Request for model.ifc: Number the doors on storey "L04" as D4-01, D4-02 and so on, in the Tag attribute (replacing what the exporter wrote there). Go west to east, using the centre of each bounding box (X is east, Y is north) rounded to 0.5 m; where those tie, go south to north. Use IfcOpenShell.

First a look at what the model holds.

```python
import ifcopenshell
import ifcopenshell.util.element
import ifcopenshell.util.placement

model = ifcopenshell.open("model.ifc")
print(model.schema)
storey = next(s for s in model.by_type("IfcBuildingStorey") if s.Name == "L04")
doors = [e for e in ifcopenshell.util.element.get_decomposition(storey) if e.is_a("IfcDoor")]
for e in sorted(doors, key=lambda e: e.id()):
    origin = ifcopenshell.util.placement.get_local_placement(e.ObjectPlacement)[:3, 3]
    print(e.id(), e.Tag, e.Name, origin.round(2) + 0.0, sep=" | ")
```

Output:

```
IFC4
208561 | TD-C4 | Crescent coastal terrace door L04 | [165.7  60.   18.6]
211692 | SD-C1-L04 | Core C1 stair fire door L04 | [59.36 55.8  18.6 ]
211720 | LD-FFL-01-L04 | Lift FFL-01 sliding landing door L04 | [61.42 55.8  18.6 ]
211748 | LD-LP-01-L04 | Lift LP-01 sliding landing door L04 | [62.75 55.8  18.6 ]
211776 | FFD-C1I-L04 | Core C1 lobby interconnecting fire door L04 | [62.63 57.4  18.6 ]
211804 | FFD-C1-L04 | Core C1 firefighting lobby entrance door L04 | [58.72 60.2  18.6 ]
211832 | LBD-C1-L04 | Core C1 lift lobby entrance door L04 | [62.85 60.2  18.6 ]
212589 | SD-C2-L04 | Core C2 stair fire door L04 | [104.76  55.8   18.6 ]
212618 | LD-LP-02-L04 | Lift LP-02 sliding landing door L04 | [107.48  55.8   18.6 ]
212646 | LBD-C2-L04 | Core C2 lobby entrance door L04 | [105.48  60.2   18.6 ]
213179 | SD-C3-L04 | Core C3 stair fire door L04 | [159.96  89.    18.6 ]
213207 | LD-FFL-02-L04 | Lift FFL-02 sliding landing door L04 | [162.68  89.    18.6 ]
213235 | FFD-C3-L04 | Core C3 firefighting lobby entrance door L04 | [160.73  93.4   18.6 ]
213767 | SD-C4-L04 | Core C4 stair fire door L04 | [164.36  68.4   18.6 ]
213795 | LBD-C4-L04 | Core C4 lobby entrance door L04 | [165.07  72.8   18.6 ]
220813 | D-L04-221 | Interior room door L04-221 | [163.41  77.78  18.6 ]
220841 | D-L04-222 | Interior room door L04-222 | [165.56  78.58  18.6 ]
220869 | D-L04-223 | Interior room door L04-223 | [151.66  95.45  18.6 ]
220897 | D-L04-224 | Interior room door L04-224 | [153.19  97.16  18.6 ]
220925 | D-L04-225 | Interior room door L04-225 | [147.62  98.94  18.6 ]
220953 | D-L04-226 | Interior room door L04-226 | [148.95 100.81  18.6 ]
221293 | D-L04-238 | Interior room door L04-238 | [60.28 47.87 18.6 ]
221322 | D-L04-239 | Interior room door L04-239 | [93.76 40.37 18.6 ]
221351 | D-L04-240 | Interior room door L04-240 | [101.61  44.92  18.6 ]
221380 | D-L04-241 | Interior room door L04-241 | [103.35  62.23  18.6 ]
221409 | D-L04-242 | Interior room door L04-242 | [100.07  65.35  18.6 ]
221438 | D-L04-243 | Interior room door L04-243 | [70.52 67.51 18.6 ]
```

```python
import ifcopenshell
import ifcopenshell.geom
import ifcopenshell.util.element
import ifcopenshell.util.shape

model = ifcopenshell.open("model.ifc")
settings = ifcopenshell.geom.settings()
settings.set("use-world-coords", True)


def centre(element):
    shape = ifcopenshell.geom.create_shape(settings, element)
    return ifcopenshell.util.shape.get_bbox_centroid(shape.geometry)


storey = next(s for s in model.by_type("IfcBuildingStorey") if s.Name == "L04")
doors = [e for e in ifcopenshell.util.element.get_decomposition(storey) if e.is_a("IfcDoor")]

# Insertion points can sit at a corner or the storey origin, so sort by the geometry (in metres).
centres = {e: centre(e) for e in doors}
doors.sort(key=lambda e: (round(centres[e][0] / 0.5), centres[e][1]))

for i, e in enumerate(doors, start=1):
    number = f"D4-{i:02d}"
    e.Tag = number
    print(e.id(), number)

model.write("model_v2.ifc")
```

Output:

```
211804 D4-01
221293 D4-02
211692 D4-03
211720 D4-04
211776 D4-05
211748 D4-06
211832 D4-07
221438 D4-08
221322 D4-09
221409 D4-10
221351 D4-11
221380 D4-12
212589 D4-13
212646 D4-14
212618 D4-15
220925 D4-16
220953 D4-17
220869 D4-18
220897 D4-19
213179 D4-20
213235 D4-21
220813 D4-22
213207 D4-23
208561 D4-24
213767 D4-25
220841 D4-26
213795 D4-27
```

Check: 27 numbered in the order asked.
